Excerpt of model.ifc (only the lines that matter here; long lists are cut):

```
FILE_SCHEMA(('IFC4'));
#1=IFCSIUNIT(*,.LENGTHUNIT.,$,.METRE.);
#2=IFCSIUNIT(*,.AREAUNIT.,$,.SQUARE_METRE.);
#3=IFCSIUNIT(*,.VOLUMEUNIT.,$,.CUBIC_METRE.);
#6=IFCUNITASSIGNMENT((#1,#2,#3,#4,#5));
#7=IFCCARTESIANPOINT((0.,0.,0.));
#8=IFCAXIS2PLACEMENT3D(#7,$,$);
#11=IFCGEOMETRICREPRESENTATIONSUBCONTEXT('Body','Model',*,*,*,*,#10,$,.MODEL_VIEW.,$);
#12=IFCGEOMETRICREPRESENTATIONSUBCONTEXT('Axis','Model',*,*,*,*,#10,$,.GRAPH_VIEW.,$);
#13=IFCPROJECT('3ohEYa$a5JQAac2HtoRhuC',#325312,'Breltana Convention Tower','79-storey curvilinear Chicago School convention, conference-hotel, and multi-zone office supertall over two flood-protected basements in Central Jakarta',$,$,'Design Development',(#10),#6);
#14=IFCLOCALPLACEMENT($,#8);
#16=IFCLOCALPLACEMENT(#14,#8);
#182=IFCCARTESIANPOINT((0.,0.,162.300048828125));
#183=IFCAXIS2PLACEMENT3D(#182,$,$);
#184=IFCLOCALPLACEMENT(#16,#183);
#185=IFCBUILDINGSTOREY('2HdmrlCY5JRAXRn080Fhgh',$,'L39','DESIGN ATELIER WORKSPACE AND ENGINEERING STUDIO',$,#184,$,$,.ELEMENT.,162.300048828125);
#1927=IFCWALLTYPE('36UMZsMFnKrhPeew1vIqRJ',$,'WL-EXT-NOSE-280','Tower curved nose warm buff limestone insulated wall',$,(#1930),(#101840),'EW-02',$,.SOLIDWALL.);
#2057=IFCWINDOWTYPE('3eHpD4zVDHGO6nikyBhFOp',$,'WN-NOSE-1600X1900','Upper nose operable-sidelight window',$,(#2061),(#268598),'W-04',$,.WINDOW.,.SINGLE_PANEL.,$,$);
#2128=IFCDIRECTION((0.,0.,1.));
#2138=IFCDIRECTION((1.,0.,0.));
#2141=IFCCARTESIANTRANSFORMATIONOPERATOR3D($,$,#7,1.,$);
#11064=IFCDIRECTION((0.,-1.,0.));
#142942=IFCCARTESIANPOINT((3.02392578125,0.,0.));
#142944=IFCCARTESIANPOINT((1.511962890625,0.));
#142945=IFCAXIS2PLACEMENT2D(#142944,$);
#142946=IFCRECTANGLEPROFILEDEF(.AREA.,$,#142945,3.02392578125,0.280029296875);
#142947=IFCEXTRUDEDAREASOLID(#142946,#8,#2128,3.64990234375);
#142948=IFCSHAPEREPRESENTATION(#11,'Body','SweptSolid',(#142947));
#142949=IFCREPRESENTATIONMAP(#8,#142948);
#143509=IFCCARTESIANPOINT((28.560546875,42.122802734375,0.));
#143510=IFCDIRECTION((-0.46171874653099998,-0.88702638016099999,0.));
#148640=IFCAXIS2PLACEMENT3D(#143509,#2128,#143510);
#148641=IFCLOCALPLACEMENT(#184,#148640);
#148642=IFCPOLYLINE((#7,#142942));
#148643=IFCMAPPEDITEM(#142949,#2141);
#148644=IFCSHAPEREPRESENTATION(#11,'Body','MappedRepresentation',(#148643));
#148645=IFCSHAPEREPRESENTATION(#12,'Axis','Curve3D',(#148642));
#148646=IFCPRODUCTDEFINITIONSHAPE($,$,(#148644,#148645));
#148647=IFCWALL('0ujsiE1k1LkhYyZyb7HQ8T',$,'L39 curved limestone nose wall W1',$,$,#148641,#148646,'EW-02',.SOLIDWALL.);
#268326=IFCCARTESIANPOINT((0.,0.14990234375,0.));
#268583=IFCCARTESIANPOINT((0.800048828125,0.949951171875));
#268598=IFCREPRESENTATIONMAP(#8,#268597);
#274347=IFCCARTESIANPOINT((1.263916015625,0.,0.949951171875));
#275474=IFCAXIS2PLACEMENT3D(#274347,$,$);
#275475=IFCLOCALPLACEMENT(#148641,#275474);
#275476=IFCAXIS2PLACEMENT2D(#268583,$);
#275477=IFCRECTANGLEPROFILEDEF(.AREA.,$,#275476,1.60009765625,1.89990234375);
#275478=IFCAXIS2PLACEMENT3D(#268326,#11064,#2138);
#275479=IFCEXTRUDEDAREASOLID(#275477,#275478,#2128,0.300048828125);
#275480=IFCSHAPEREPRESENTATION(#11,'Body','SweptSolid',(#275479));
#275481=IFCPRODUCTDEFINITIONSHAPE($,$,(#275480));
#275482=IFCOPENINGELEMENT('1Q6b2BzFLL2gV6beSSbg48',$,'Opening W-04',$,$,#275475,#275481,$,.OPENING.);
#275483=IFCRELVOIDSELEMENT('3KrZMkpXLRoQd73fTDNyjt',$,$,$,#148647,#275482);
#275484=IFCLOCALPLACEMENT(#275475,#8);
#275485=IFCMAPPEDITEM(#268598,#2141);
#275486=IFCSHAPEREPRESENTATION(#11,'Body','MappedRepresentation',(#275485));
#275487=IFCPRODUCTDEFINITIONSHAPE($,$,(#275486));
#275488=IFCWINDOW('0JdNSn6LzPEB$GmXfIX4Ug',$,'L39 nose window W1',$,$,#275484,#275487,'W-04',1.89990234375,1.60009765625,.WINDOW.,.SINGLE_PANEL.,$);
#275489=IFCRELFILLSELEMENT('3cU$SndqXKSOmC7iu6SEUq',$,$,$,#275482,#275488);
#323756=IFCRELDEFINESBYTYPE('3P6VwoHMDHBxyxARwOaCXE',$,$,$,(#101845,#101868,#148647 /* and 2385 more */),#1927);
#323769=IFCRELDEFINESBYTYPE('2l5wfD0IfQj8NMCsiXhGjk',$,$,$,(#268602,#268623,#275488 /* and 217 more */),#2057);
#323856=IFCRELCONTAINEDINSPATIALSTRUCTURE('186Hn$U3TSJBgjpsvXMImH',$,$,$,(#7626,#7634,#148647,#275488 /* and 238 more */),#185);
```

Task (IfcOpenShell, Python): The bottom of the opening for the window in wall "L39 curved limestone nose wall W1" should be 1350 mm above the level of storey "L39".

```python
import numpy as np
import ifcopenshell
import ifcopenshell.api.geometry
import ifcopenshell.geom
import ifcopenshell.util.element
import ifcopenshell.util.placement
import ifcopenshell.util.shape
import ifcopenshell.util.unit

model = ifcopenshell.open("model.ifc")
unit_scale = ifcopenshell.util.unit.calculate_unit_scale(model)

window = model.by_guid("0JdNSn6LzPEB$GmXfIX4Ug")
opening = window.FillsVoids[0].RelatingOpeningElement
storey = ifcopenshell.util.element.get_container(window, ifc_class="IfcBuildingStorey")
level = ifcopenshell.util.placement.get_local_placement(storey.ObjectPlacement)[2, 3]

# The opening's origin need not be at the sill, so measure its lowest point.
shape = ifcopenshell.geom.create_shape(ifcopenshell.geom.settings(), opening)
bottom = ifcopenshell.util.shape.get_shape_bottom_elevation(shape, shape.geometry) / unit_scale
dz = level + 1.35 / unit_scale - bottom

shift = np.array([0.0, 0.0, dz])
# The window is placed relative to its opening, so it follows when the opening moves.
matrix = ifcopenshell.util.placement.get_local_placement(opening.ObjectPlacement)
matrix[:3, 3] += shift
ifcopenshell.api.geometry.edit_object_placement(
    model, product=opening, matrix=matrix, is_si=False, should_transform_children=True
)

print(f"moved by {dz * unit_scale:+.3f} m")

model.write("model_updated.ifc")
```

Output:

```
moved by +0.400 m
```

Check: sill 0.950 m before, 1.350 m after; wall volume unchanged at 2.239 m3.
